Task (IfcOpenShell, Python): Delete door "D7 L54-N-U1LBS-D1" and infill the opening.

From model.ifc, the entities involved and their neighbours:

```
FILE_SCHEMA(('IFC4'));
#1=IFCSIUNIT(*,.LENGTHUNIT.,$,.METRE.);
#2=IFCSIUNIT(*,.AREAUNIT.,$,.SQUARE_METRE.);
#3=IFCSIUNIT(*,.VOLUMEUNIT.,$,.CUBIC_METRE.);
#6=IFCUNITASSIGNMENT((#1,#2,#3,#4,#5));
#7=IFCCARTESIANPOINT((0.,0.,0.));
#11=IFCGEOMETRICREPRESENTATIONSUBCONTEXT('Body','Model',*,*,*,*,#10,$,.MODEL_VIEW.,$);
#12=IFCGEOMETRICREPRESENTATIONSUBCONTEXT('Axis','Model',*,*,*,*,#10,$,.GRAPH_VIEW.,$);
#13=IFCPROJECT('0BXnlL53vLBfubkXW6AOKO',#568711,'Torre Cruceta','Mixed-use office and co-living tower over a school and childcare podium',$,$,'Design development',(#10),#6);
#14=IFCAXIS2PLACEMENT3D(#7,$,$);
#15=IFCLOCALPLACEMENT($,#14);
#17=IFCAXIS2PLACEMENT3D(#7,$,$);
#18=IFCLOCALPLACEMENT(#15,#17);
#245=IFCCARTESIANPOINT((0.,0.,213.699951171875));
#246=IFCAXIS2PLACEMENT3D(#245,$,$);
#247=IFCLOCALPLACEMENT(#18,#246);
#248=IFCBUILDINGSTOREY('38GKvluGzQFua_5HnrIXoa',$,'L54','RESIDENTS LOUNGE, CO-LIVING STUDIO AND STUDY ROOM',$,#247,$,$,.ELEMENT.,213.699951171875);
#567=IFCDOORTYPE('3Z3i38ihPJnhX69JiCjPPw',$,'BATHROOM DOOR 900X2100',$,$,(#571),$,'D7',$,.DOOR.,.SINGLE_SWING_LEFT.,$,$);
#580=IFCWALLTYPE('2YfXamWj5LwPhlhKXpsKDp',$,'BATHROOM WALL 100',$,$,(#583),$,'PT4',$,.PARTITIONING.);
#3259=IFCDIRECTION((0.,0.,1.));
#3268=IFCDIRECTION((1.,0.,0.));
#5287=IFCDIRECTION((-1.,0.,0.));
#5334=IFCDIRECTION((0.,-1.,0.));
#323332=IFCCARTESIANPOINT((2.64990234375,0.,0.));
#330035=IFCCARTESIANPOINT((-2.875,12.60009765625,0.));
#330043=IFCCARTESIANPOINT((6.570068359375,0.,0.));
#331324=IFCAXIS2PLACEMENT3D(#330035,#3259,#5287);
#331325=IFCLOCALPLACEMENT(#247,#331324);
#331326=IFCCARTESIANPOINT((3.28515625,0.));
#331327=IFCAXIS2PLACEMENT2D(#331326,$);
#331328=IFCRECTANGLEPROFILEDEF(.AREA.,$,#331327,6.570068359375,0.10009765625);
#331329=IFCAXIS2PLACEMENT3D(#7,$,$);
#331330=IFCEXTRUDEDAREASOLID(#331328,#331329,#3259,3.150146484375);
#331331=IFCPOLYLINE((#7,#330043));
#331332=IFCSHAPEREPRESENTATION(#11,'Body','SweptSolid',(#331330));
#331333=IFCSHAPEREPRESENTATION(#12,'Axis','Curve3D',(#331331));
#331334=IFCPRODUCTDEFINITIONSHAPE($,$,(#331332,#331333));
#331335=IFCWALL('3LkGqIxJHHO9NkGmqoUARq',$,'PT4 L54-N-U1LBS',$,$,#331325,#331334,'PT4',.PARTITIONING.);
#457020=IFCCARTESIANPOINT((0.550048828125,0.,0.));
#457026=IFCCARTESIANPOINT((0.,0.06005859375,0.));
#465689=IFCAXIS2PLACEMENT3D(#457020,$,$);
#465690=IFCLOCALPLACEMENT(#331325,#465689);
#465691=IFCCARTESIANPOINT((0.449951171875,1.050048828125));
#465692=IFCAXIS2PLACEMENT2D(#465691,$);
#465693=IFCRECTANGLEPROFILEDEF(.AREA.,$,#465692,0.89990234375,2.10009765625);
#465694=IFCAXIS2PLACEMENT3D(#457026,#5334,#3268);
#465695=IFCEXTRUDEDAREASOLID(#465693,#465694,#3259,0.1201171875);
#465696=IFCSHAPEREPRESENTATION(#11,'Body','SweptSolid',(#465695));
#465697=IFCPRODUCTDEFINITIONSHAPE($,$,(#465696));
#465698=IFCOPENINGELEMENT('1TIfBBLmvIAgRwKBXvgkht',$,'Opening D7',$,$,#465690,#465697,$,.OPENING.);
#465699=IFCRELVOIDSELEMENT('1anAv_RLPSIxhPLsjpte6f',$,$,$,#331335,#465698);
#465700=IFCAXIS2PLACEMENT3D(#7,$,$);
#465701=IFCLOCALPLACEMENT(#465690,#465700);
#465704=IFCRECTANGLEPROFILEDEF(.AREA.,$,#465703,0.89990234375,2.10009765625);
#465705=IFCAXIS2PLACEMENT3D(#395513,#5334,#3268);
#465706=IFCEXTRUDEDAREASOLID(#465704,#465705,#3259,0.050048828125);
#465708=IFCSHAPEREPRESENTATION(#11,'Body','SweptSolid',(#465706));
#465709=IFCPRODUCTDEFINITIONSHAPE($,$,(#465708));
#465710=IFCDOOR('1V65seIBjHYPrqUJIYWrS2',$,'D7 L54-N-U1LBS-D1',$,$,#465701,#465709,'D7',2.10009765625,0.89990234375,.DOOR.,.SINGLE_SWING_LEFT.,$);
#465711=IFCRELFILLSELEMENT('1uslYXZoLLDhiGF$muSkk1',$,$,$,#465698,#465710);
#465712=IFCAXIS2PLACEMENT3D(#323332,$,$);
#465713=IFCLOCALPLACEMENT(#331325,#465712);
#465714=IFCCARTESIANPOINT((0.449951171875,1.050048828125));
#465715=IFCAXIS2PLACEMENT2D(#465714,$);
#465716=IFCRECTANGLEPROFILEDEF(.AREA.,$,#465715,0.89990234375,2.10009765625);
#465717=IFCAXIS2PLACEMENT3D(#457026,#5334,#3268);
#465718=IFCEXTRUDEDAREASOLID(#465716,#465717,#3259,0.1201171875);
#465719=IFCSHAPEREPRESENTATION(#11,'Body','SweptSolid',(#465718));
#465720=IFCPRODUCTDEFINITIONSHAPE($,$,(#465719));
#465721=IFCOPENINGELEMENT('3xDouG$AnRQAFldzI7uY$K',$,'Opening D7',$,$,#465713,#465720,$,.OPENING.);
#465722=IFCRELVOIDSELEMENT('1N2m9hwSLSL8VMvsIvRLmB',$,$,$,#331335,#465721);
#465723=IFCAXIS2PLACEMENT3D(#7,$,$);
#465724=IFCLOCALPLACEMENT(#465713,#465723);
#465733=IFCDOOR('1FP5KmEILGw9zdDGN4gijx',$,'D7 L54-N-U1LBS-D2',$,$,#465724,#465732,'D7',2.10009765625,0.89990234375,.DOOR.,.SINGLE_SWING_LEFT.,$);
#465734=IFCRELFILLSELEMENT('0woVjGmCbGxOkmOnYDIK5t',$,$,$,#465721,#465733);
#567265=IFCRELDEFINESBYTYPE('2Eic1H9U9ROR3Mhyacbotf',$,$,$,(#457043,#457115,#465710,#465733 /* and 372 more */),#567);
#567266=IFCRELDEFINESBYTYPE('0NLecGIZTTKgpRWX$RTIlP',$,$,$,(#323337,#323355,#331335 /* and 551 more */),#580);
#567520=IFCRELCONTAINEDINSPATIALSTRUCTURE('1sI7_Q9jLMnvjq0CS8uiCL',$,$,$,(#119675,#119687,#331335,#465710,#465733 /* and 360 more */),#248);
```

```python
import ifcopenshell
import ifcopenshell.api.feature
import ifcopenshell.api.root
import ifcopenshell.geom
import ifcopenshell.util.shape

model = ifcopenshell.open("model.ifc")
settings = ifcopenshell.geom.settings()


def volume(element):
    """Net volume in cubic metres, openings subtracted."""
    shape = ifcopenshell.geom.create_shape(settings, element)
    return ifcopenshell.util.shape.get_volume(shape.geometry)


door = model.by_guid("1V65seIBjHYPrqUJIYWrS2")
opening = door.FillsVoids[0].RelatingOpeningElement
wall = opening.VoidsElements[0].RelatingBuildingElement
before = volume(wall)

ifcopenshell.api.root.remove_product(model, product=door)
ifcopenshell.api.feature.remove_feature(model, feature=opening)

after = volume(wall)

print(f"wall volume {before:.3f} -> {after:.3f} m3")

model.write("model_edited.ifc")
```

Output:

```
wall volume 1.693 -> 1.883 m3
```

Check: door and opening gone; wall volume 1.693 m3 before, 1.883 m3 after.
